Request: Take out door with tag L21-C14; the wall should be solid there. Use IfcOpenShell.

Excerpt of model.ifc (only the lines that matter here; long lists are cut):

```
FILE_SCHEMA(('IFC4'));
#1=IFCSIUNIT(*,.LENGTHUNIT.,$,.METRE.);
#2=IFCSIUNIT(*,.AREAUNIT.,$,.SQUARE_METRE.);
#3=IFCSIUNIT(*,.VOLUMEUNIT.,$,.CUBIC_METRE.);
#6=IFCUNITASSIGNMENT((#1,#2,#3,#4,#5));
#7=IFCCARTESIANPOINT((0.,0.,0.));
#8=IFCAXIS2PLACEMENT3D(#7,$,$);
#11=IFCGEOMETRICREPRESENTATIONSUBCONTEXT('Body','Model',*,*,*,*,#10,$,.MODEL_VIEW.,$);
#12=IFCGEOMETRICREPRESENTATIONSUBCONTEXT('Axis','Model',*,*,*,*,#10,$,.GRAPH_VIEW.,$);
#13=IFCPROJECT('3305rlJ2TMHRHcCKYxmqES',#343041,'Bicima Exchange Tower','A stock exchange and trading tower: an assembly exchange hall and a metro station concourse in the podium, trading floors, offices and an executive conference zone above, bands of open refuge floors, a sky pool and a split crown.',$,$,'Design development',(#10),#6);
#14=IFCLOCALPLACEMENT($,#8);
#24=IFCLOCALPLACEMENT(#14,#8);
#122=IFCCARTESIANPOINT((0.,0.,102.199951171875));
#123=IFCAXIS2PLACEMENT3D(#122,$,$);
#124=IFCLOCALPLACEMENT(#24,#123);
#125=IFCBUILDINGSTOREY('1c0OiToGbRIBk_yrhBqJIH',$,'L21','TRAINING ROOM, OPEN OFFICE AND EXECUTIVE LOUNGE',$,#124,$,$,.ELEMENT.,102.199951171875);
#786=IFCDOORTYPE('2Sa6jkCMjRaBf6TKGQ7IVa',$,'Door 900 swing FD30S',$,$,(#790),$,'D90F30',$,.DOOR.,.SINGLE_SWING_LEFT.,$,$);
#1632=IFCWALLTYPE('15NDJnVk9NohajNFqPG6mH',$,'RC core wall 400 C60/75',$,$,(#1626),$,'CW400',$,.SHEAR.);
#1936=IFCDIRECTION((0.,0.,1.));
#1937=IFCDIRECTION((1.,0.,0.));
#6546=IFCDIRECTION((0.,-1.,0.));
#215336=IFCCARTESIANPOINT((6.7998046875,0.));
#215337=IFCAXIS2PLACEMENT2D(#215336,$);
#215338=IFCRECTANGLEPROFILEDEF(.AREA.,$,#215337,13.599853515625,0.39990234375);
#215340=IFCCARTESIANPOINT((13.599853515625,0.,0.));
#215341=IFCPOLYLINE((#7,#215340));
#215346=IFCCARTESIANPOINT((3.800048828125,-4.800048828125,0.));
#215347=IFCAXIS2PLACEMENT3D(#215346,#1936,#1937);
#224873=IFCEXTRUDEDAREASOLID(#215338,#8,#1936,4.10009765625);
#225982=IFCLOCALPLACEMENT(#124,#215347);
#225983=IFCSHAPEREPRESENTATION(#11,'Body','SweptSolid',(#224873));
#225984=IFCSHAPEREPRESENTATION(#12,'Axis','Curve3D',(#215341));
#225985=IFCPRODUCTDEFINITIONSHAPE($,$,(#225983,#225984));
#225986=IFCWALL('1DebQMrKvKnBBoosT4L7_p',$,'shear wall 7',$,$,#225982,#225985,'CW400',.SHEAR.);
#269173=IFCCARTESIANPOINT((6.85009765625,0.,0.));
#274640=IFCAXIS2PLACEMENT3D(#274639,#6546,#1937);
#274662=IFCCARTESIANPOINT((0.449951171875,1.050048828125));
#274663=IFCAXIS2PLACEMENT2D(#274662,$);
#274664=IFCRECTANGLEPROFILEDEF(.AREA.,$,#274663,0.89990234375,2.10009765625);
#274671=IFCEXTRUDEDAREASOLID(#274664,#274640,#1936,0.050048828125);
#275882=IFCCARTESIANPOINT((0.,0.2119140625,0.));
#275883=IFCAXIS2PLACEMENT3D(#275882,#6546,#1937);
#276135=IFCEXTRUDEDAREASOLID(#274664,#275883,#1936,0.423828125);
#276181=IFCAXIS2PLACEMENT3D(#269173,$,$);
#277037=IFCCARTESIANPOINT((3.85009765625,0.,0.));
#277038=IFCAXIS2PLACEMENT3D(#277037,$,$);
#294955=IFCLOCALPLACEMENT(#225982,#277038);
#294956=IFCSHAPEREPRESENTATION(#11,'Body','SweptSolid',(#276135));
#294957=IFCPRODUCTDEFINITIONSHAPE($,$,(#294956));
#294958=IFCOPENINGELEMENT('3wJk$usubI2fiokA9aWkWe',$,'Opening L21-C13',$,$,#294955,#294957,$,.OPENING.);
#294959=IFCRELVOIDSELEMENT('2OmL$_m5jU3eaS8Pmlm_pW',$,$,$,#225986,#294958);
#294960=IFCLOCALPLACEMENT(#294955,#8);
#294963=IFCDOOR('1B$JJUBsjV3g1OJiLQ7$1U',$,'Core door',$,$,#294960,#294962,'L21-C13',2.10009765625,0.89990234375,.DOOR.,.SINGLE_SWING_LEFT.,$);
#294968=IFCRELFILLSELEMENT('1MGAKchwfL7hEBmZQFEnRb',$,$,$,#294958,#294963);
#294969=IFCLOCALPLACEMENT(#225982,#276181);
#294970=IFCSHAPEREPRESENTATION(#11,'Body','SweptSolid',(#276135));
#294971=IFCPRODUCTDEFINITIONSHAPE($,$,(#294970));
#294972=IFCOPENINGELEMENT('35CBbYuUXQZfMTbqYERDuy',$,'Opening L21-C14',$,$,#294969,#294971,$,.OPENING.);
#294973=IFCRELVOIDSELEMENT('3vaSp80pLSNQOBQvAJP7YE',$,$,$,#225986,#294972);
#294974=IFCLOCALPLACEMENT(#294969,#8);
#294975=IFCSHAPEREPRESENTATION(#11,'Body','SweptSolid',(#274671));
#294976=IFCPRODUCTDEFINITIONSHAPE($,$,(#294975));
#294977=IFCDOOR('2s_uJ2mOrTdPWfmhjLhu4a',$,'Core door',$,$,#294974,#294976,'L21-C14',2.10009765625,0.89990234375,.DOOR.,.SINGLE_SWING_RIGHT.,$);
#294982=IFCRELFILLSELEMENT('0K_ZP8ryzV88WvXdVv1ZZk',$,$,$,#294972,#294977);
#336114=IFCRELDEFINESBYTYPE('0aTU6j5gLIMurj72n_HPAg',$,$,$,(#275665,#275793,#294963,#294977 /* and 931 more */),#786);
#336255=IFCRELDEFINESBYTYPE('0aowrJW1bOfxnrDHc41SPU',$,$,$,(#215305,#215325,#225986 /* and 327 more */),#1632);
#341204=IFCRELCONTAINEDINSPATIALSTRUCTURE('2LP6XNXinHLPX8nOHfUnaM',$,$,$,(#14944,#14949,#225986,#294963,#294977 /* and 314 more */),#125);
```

```python
import ifcopenshell
import ifcopenshell.api.feature
import ifcopenshell.api.root
import ifcopenshell.geom
import ifcopenshell.util.shape

model = ifcopenshell.open("model.ifc")
settings = ifcopenshell.geom.settings()


def volume(element):
    """Net volume in cubic metres, openings subtracted."""
    shape = ifcopenshell.geom.create_shape(settings, element)
    return ifcopenshell.util.shape.get_volume(shape.geometry)


door = model.by_id(294977)
opening = door.FillsVoids[0].RelatingOpeningElement
wall = opening.VoidsElements[0].RelatingBuildingElement
before = volume(wall)

ifcopenshell.api.root.remove_product(model, product=door)
ifcopenshell.api.feature.remove_feature(model, feature=opening)

after = volume(wall)

print(f"wall volume {before:.3f} -> {after:.3f} m3")

model.write("model_updated.ifc")
```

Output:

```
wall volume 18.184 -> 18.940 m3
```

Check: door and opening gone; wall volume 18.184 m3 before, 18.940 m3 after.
